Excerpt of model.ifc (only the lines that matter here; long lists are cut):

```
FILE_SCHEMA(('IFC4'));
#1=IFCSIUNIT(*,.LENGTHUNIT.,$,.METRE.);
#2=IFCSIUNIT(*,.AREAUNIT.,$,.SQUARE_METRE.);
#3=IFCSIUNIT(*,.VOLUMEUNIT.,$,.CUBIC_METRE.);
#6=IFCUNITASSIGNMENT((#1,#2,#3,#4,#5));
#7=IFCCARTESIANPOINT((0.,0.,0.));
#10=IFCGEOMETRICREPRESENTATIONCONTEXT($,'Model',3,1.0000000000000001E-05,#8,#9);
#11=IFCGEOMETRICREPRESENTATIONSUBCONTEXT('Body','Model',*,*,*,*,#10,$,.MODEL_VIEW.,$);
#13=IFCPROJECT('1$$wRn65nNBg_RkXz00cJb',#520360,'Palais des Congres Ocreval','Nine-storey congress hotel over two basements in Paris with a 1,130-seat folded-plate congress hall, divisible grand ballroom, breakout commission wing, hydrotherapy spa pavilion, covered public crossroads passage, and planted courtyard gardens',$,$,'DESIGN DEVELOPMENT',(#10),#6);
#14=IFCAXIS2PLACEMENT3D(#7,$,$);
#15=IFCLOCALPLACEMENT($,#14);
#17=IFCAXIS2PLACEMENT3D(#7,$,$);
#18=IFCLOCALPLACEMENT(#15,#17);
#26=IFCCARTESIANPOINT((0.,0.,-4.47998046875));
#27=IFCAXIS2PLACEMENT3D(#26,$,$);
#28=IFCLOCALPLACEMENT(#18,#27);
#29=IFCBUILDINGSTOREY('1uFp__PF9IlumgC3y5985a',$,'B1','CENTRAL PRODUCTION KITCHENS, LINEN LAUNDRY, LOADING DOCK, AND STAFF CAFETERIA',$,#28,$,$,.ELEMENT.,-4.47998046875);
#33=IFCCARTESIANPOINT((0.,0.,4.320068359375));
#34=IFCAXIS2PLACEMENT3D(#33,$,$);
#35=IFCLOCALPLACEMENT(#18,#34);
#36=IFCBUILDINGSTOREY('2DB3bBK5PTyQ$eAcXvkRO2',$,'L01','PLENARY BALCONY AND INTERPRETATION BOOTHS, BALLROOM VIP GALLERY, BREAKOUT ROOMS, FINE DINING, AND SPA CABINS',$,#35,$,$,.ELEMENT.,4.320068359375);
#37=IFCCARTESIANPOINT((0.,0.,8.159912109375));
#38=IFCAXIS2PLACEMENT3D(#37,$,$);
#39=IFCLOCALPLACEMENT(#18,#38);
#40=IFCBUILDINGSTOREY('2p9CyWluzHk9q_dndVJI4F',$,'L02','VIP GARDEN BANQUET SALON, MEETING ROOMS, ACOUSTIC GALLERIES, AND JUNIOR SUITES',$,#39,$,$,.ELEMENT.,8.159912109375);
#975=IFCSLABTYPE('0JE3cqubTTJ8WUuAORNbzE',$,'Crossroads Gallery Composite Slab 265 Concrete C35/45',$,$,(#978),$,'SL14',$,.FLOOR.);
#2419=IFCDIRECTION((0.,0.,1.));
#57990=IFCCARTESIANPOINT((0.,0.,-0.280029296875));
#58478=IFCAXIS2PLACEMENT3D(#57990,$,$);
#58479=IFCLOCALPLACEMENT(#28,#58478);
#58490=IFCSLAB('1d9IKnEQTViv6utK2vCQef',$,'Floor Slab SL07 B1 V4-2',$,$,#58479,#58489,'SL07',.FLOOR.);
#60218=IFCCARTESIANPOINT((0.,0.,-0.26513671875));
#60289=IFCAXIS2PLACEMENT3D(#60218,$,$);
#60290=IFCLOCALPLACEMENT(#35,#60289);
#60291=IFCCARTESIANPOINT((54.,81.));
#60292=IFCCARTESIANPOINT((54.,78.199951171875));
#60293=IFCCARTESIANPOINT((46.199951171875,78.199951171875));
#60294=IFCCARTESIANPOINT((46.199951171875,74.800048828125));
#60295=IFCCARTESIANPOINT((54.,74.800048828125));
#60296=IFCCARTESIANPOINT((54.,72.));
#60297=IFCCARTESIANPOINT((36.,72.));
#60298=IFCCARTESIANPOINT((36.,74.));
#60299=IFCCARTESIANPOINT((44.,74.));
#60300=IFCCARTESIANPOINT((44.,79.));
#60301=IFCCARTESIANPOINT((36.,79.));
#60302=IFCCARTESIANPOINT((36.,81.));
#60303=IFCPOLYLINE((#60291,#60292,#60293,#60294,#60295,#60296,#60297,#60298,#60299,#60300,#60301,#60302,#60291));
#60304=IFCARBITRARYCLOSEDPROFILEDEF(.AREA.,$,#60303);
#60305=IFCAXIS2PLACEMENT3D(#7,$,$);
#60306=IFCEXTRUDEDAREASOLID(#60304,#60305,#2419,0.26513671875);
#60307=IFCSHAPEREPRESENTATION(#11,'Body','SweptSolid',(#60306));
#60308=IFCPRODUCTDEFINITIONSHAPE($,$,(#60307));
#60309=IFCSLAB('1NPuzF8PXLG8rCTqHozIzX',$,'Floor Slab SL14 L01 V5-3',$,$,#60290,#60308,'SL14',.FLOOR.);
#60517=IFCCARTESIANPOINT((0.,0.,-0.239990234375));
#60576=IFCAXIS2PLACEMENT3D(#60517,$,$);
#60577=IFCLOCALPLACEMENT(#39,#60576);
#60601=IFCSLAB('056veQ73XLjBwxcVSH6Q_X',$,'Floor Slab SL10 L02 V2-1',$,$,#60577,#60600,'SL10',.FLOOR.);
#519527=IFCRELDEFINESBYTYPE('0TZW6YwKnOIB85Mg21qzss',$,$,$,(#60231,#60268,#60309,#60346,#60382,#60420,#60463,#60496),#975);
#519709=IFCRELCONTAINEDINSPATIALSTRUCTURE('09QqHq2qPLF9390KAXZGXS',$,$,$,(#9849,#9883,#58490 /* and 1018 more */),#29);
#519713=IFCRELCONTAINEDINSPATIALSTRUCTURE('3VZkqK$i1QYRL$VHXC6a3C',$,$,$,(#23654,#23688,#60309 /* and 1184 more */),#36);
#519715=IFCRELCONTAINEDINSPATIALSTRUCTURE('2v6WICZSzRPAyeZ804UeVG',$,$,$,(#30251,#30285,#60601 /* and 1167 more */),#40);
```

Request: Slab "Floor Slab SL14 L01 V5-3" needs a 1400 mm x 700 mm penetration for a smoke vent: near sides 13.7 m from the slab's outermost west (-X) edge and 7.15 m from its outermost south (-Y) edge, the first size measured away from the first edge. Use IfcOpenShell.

```python
import numpy as np
import ifcopenshell
import ifcopenshell.api.feature
import ifcopenshell.api.geometry
import ifcopenshell.api.root
import ifcopenshell.geom
import ifcopenshell.util.placement
import ifcopenshell.util.representation
import ifcopenshell.util.shape
import ifcopenshell.util.unit

model = ifcopenshell.open("model.ifc")
unit_scale = ifcopenshell.util.unit.calculate_unit_scale(model)
settings = ifcopenshell.geom.settings()


def volume(element):
    """Net volume in cubic metres, openings subtracted."""
    shape = ifcopenshell.geom.create_shape(settings, element)
    return ifcopenshell.util.shape.get_volume(shape.geometry)


slab = model.by_id(60309)
before = volume(slab)

# Extent in the slab's own axes, in metres. The edges named are its -X and -Y sides.
slab_shape = ifcopenshell.geom.create_shape(settings, slab)
vertices = ifcopenshell.util.shape.get_vertices(slab_shape.geometry)
x_min, y_min, bottom = vertices.min(axis=0)
top = vertices[:, 2].max()

opening = ifcopenshell.api.root.create_entity(model, ifc_class="IfcOpeningElement", name="Smoke vent opening", predefined_type="OPENING")
context = ifcopenshell.util.representation.get_context(model, "Model", "Body", "MODEL_VIEW")
width, depth = 1.4, 0.7
outline = [(0.0, 0.0), (width, 0.0), (width, depth), (0.0, depth), (0.0, 0.0)]
# Overshoot both faces by 50 mm so the cut is clean.
shape = ifcopenshell.api.geometry.add_slab_representation(
    model, context=context, depth=top - bottom + 0.1, polyline=outline
)
ifcopenshell.api.geometry.assign_representation(model, product=opening, representation=shape)

matrix = ifcopenshell.util.placement.get_local_placement(slab.ObjectPlacement)
matrix[:, 3] = matrix @ np.append(np.array([x_min + 13.7, y_min + 7.15, bottom - 0.05]) / unit_scale, 1.0)
ifcopenshell.api.geometry.edit_object_placement(model, product=opening, matrix=matrix, is_si=False)
ifcopenshell.api.feature.add_feature(model, feature=opening, element=slab)

after = volume(slab)

print(f"slab volume {before:.3f} -> {after:.3f} m3")

model.write("model_v2.ifc")
```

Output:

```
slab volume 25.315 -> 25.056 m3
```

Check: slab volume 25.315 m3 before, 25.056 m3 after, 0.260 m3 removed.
